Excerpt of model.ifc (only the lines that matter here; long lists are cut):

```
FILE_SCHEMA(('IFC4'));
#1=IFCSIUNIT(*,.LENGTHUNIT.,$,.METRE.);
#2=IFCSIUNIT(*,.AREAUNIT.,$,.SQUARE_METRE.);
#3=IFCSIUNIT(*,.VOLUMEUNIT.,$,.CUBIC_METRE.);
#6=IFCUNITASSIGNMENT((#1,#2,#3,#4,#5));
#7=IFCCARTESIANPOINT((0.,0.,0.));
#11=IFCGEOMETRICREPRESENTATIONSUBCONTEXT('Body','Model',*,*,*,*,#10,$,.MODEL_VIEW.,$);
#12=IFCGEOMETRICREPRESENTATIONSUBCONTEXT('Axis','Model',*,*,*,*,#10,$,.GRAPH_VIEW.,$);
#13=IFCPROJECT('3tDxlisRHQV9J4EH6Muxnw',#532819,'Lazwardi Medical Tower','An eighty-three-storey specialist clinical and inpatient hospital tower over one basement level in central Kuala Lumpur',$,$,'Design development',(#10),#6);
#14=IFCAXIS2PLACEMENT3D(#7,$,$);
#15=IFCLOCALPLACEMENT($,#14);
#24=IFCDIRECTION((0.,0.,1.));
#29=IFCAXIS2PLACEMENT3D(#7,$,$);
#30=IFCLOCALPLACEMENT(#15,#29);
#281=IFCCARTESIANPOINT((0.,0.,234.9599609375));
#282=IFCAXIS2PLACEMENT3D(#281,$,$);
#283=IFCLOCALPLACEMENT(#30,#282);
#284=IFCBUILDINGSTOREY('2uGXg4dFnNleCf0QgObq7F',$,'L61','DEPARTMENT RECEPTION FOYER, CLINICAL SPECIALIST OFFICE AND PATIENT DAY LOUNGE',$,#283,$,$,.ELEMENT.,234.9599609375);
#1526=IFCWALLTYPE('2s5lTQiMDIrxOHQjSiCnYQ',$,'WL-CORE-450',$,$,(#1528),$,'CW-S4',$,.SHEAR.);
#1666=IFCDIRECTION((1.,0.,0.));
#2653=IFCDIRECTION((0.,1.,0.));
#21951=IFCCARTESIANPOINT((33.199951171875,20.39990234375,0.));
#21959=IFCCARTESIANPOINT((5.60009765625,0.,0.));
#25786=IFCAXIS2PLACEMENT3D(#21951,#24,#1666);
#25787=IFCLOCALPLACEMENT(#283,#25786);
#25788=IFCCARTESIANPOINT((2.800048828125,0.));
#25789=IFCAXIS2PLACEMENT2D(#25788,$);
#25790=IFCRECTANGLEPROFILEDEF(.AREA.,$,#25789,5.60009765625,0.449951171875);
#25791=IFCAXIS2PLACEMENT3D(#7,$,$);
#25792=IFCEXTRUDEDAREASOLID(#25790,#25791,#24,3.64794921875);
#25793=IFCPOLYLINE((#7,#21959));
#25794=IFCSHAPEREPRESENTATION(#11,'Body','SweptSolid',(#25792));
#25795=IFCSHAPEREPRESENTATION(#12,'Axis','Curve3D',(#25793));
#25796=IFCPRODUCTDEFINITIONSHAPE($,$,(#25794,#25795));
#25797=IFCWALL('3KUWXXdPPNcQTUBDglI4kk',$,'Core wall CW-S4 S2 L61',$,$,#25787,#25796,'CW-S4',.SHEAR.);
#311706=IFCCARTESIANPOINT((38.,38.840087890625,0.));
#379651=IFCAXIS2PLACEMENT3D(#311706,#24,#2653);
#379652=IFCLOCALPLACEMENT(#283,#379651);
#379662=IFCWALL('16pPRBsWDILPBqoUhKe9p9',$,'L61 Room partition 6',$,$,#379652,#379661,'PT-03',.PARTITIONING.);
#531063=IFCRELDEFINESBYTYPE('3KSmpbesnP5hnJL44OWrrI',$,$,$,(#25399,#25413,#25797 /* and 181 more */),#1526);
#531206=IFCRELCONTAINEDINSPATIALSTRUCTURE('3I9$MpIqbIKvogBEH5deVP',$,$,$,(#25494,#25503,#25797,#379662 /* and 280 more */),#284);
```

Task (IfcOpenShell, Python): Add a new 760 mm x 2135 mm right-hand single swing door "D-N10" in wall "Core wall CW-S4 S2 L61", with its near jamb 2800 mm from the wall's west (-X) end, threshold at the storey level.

```python
import numpy as np
import ifcopenshell
import ifcopenshell.api.feature
import ifcopenshell.api.geometry
import ifcopenshell.api.root
import ifcopenshell.api.spatial
import ifcopenshell.geom
import ifcopenshell.util.element
import ifcopenshell.util.placement
import ifcopenshell.util.representation
import ifcopenshell.util.shape
import ifcopenshell.util.unit

model = ifcopenshell.open("model.ifc")
unit_scale = ifcopenshell.util.unit.calculate_unit_scale(model)
settings = ifcopenshell.geom.settings()


def volume(element):
    """Net volume in cubic metres, openings subtracted."""
    shape = ifcopenshell.geom.create_shape(settings, element)
    return ifcopenshell.util.shape.get_volume(shape.geometry)


wall = model.by_guid("3KUWXXdPPNcQTUBDglI4kk")
storey = ifcopenshell.util.element.get_container(wall, ifc_class="IfcBuildingStorey")
context = ifcopenshell.util.representation.get_context(model, "Model", "Body", "MODEL_VIEW")
before = volume(wall)

width, height, from_end, sill = 0.76, 2.135, 2.8, 0.0  # metres

# The wall runs along its own X axis, and the end named is its -X end.
wall_shape = ifcopenshell.geom.create_shape(settings, wall)
x, y, z = ifcopenshell.util.shape.get_vertices(wall_shape.geometry).T
start = x.min() + from_end
face, thickness = float(y.min()), float(y.max() - y.min())
wall_matrix = ifcopenshell.util.placement.get_local_placement(wall.ObjectPlacement)
level = ifcopenshell.util.placement.get_local_placement(storey.ObjectPlacement)[2, 3]


def in_wall(x, y):
    """Placement at x, y metres in the wall's axes, at sill height."""
    matrix = wall_matrix.copy()
    matrix[:, 3] = wall_matrix @ np.array([x / unit_scale, y / unit_scale, 0.0, 1.0])
    matrix[2, 3] = level + sill / unit_scale
    return matrix


# Opening: a box that overshoots both wall faces by 50 mm.
opening = ifcopenshell.api.root.create_entity(model, ifc_class="IfcOpeningElement", predefined_type="OPENING")
box = ifcopenshell.api.geometry.add_wall_representation(
    model, context=context, length=width, height=height, thickness=thickness + 0.1
)
ifcopenshell.api.geometry.assign_representation(model, product=opening, representation=box)
ifcopenshell.api.geometry.edit_object_placement(model, product=opening, matrix=in_wall(start, face - 0.05), is_si=False)
ifcopenshell.api.feature.add_feature(model, feature=opening, element=wall)

door = ifcopenshell.api.root.create_entity(model, ifc_class="IfcDoor", name="D-N10", predefined_type="DOOR")
door.OverallWidth, door.OverallHeight = width / unit_scale, height / unit_scale
door.OperationType = "SINGLE_SWING_RIGHT"
body = ifcopenshell.api.geometry.add_door_representation(
    model,
    context=context,
    overall_width=door.OverallWidth,
    overall_height=door.OverallHeight,
    operation_type="SINGLE_SWING_RIGHT",
    lining_properties={"LiningDepth": thickness / unit_scale, "ThresholdDepth": thickness / unit_scale},
)
ifcopenshell.api.geometry.assign_representation(model, product=door, representation=body)
ifcopenshell.api.spatial.assign_container(model, products=[door], relating_structure=storey)
ifcopenshell.api.feature.add_filling(model, opening=opening, element=door)

# The lining spans the wall, so the door starts at the wall face.
ifcopenshell.api.geometry.edit_object_placement(model, product=door, matrix=in_wall(start, face), is_si=False)

after = volume(wall)

print(f"wall volume {before:.3f} -> {after:.3f} m3")

model.write("model-out.ifc")
```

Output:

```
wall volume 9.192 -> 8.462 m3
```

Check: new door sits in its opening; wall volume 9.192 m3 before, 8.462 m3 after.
